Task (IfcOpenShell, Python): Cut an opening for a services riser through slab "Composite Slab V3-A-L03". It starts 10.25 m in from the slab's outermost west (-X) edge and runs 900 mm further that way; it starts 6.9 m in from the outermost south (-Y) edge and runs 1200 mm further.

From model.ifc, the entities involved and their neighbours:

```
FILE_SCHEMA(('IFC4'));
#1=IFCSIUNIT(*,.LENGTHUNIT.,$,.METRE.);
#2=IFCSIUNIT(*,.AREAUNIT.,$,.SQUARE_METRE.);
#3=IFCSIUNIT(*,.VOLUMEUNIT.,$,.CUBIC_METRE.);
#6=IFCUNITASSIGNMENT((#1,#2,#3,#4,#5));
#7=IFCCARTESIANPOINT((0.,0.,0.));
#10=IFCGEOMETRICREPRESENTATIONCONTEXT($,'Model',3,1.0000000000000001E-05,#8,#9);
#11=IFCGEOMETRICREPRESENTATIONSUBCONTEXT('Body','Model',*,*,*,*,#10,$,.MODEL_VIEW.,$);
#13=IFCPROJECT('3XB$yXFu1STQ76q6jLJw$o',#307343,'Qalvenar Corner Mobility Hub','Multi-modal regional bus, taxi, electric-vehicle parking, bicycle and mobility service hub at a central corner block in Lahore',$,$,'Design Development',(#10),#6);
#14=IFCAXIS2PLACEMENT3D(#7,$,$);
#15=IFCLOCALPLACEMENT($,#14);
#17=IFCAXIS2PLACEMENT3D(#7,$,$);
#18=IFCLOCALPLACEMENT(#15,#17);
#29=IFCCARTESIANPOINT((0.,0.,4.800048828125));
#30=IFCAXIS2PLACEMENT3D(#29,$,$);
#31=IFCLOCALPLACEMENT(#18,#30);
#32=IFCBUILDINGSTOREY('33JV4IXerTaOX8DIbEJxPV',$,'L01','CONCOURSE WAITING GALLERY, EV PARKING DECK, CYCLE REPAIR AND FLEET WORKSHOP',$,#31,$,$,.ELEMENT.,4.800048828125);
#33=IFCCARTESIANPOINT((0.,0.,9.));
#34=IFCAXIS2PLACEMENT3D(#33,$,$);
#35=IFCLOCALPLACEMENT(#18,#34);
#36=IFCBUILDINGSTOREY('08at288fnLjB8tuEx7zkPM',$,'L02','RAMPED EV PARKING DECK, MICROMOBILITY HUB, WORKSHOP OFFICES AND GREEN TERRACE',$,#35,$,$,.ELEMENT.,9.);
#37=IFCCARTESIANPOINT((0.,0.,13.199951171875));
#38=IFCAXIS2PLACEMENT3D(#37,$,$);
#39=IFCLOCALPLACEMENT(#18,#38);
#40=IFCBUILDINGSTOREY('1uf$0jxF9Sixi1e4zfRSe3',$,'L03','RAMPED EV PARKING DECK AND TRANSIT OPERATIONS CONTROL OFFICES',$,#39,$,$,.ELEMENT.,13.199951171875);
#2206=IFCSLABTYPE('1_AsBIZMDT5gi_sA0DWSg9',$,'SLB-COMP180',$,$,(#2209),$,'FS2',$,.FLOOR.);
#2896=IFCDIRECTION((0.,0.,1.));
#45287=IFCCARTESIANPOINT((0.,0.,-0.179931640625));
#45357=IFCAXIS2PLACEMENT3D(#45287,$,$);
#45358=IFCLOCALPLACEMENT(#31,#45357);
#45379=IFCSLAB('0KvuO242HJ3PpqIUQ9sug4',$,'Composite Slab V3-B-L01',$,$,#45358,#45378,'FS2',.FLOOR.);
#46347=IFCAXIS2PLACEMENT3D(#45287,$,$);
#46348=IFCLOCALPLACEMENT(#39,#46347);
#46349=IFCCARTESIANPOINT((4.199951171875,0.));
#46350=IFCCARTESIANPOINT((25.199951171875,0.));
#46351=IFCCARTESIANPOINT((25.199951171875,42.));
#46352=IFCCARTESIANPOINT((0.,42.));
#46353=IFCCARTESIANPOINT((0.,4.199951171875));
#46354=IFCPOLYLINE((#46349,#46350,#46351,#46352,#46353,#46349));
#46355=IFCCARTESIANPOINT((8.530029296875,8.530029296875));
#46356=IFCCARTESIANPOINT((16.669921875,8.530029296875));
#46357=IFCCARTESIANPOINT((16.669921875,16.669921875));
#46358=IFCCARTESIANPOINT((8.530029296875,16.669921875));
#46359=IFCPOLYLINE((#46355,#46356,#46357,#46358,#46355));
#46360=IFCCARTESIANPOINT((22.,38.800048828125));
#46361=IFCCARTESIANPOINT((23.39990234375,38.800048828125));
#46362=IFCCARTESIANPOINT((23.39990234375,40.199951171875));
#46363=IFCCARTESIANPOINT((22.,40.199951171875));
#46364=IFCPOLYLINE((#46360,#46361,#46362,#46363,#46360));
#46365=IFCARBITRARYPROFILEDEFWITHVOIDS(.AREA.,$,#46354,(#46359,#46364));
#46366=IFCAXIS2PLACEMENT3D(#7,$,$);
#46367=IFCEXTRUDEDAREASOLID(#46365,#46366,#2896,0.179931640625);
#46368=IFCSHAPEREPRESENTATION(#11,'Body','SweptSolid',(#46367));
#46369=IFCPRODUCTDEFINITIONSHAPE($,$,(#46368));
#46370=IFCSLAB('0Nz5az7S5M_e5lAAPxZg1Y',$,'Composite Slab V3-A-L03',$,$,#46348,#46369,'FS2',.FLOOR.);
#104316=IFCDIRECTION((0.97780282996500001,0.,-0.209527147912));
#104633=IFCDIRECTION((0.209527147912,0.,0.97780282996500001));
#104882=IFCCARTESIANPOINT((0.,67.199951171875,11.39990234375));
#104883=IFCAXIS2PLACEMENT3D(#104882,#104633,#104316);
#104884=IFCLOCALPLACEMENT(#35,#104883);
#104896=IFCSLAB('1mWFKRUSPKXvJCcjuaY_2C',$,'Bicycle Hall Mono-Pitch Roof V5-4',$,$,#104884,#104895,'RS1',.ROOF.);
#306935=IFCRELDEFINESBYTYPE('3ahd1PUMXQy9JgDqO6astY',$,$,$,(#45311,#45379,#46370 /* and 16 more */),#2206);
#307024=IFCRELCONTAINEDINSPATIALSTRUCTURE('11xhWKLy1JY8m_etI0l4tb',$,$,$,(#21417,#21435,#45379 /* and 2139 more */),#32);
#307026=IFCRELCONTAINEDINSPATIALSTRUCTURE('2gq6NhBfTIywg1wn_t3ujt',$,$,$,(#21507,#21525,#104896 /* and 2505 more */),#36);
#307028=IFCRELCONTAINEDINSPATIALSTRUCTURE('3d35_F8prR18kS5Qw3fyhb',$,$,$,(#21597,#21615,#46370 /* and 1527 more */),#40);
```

```python
import numpy as np
import ifcopenshell
import ifcopenshell.api.feature
import ifcopenshell.api.geometry
import ifcopenshell.api.root
import ifcopenshell.geom
import ifcopenshell.util.placement
import ifcopenshell.util.representation
import ifcopenshell.util.shape
import ifcopenshell.util.unit

model = ifcopenshell.open("model.ifc")
unit_scale = ifcopenshell.util.unit.calculate_unit_scale(model)
settings = ifcopenshell.geom.settings()


def volume(element):
    """Net volume in cubic metres, openings subtracted."""
    shape = ifcopenshell.geom.create_shape(settings, element)
    return ifcopenshell.util.shape.get_volume(shape.geometry)


slab = model.by_guid("0Nz5az7S5M_e5lAAPxZg1Y")
before = volume(slab)

# Extent in the slab's own axes, in metres. The edges named are its -X and -Y sides.
slab_shape = ifcopenshell.geom.create_shape(settings, slab)
vertices = ifcopenshell.util.shape.get_vertices(slab_shape.geometry)
x_min, y_min, bottom = vertices.min(axis=0)
top = vertices[:, 2].max()

opening = ifcopenshell.api.root.create_entity(model, ifc_class="IfcOpeningElement", name="Services riser opening", predefined_type="OPENING")
context = ifcopenshell.util.representation.get_context(model, "Model", "Body", "MODEL_VIEW")
width, depth = 0.9, 1.2
outline = [(0.0, 0.0), (width, 0.0), (width, depth), (0.0, depth), (0.0, 0.0)]
# Overshoot both faces by 50 mm so the cut is clean.
shape = ifcopenshell.api.geometry.add_slab_representation(
    model, context=context, depth=top - bottom + 0.1, polyline=outline
)
ifcopenshell.api.geometry.assign_representation(model, product=opening, representation=shape)

matrix = ifcopenshell.util.placement.get_local_placement(slab.ObjectPlacement)
matrix[:, 3] = matrix @ np.append(np.array([x_min + 10.25, y_min + 6.9, bottom - 0.05]) / unit_scale, 1.0)
ifcopenshell.api.geometry.edit_object_placement(model, product=opening, matrix=matrix, is_si=False)
ifcopenshell.api.feature.add_feature(model, feature=opening, element=slab)

after = volume(slab)

print(f"slab volume {before:.3f} -> {after:.3f} m3")

model.write("model_edited.ifc")
```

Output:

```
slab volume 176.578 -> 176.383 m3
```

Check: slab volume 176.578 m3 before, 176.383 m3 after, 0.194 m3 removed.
